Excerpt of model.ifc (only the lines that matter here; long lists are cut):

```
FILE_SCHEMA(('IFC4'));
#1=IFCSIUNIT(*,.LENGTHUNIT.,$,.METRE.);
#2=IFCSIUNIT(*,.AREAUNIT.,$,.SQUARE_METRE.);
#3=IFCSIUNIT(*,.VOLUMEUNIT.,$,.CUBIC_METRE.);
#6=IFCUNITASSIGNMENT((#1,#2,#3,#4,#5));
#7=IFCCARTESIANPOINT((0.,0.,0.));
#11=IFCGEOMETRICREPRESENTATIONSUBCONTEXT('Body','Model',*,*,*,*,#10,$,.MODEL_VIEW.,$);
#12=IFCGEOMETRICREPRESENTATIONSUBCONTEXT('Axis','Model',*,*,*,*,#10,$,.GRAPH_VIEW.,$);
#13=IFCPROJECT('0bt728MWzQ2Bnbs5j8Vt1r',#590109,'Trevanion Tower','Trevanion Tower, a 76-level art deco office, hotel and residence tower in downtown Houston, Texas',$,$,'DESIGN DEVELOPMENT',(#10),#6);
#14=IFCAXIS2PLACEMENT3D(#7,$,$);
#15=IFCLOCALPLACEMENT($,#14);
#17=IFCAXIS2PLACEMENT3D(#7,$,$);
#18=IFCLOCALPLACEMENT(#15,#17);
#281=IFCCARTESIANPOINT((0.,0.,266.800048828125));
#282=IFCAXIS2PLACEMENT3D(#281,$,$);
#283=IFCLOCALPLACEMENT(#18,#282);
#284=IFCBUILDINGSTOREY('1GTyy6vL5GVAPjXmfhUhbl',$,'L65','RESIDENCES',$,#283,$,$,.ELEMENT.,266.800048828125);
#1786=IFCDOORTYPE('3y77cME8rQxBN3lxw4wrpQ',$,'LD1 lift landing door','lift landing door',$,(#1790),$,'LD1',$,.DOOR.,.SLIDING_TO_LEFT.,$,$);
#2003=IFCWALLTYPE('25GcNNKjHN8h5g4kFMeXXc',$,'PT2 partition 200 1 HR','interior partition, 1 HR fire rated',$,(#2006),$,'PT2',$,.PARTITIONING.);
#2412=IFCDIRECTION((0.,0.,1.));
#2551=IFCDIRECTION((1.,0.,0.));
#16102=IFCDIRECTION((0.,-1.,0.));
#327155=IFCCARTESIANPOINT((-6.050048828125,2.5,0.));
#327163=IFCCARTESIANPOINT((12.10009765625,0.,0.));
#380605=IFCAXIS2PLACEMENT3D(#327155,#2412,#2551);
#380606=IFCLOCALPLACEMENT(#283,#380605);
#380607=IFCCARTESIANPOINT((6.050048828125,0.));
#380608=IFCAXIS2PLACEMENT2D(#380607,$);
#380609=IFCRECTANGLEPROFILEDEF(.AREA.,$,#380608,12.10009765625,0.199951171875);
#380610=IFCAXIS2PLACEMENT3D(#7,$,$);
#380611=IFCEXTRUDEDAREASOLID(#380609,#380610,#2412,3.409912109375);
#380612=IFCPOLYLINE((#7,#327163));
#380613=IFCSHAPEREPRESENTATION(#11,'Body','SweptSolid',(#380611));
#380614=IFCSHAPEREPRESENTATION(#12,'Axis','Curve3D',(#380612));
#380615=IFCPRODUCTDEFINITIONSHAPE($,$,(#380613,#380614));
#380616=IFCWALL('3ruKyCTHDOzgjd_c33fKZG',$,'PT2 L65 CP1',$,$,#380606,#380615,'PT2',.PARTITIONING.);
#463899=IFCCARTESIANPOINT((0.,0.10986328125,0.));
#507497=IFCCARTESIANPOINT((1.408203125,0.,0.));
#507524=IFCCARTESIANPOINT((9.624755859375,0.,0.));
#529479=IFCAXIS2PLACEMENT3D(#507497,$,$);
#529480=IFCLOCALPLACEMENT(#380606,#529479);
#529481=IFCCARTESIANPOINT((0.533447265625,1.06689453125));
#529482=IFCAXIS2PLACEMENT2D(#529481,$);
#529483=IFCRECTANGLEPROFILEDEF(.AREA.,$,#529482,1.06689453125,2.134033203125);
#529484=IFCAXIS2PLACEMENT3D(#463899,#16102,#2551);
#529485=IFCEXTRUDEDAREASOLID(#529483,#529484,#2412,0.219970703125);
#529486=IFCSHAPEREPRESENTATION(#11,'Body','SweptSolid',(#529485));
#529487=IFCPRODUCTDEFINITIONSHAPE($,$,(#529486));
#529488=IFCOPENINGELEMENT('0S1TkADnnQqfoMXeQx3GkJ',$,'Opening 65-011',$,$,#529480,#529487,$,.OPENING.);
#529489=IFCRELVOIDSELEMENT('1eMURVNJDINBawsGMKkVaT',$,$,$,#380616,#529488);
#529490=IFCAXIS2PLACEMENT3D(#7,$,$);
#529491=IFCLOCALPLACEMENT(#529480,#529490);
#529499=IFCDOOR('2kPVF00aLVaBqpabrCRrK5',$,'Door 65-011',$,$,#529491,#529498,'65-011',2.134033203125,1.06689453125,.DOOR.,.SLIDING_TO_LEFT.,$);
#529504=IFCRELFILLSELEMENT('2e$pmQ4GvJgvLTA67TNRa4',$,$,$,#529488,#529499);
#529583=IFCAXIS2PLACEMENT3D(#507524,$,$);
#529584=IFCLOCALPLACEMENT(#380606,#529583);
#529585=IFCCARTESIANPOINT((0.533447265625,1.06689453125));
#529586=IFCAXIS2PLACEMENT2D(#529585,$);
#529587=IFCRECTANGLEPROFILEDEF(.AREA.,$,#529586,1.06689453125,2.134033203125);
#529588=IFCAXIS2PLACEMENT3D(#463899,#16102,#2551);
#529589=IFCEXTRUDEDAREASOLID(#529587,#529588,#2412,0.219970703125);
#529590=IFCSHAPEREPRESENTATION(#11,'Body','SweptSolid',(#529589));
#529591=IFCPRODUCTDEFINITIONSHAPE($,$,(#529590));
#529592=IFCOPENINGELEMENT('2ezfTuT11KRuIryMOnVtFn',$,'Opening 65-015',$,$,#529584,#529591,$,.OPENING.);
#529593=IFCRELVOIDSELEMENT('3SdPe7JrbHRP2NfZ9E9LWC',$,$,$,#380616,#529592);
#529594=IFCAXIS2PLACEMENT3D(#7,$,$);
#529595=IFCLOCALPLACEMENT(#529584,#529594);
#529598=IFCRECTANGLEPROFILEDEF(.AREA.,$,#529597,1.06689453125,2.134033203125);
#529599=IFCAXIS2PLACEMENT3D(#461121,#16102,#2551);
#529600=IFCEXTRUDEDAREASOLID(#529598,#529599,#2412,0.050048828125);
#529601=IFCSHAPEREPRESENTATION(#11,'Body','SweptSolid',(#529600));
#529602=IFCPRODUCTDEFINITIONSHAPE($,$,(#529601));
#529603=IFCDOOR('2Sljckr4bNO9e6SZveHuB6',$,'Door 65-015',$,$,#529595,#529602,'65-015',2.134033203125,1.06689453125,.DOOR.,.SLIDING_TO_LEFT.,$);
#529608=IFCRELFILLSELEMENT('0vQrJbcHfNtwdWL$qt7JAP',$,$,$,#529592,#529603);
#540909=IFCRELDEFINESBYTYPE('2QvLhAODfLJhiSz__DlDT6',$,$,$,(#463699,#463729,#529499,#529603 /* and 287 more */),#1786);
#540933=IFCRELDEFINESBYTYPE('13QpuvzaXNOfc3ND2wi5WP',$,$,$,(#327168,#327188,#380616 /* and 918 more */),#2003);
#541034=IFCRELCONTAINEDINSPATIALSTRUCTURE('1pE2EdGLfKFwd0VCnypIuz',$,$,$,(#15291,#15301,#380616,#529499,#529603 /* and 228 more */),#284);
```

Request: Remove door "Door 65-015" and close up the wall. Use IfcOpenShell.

```python
import ifcopenshell
import ifcopenshell.api.feature
import ifcopenshell.api.root
import ifcopenshell.geom
import ifcopenshell.util.shape

model = ifcopenshell.open("model.ifc")
settings = ifcopenshell.geom.settings()


def volume(element):
    """Net volume in cubic metres, openings subtracted."""
    shape = ifcopenshell.geom.create_shape(settings, element)
    return ifcopenshell.util.shape.get_volume(shape.geometry)


door = model.by_guid("2Sljckr4bNO9e6SZveHuB6")
opening = door.FillsVoids[0].RelatingOpeningElement
wall = opening.VoidsElements[0].RelatingBuildingElement
before = volume(wall)

ifcopenshell.api.root.remove_product(model, product=door)
ifcopenshell.api.feature.remove_feature(model, feature=opening)

after = volume(wall)

print(f"wall volume {before:.3f} -> {after:.3f} m3")

model.write("model_v2.ifc")
```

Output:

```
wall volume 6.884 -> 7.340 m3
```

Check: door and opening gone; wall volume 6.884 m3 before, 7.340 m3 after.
